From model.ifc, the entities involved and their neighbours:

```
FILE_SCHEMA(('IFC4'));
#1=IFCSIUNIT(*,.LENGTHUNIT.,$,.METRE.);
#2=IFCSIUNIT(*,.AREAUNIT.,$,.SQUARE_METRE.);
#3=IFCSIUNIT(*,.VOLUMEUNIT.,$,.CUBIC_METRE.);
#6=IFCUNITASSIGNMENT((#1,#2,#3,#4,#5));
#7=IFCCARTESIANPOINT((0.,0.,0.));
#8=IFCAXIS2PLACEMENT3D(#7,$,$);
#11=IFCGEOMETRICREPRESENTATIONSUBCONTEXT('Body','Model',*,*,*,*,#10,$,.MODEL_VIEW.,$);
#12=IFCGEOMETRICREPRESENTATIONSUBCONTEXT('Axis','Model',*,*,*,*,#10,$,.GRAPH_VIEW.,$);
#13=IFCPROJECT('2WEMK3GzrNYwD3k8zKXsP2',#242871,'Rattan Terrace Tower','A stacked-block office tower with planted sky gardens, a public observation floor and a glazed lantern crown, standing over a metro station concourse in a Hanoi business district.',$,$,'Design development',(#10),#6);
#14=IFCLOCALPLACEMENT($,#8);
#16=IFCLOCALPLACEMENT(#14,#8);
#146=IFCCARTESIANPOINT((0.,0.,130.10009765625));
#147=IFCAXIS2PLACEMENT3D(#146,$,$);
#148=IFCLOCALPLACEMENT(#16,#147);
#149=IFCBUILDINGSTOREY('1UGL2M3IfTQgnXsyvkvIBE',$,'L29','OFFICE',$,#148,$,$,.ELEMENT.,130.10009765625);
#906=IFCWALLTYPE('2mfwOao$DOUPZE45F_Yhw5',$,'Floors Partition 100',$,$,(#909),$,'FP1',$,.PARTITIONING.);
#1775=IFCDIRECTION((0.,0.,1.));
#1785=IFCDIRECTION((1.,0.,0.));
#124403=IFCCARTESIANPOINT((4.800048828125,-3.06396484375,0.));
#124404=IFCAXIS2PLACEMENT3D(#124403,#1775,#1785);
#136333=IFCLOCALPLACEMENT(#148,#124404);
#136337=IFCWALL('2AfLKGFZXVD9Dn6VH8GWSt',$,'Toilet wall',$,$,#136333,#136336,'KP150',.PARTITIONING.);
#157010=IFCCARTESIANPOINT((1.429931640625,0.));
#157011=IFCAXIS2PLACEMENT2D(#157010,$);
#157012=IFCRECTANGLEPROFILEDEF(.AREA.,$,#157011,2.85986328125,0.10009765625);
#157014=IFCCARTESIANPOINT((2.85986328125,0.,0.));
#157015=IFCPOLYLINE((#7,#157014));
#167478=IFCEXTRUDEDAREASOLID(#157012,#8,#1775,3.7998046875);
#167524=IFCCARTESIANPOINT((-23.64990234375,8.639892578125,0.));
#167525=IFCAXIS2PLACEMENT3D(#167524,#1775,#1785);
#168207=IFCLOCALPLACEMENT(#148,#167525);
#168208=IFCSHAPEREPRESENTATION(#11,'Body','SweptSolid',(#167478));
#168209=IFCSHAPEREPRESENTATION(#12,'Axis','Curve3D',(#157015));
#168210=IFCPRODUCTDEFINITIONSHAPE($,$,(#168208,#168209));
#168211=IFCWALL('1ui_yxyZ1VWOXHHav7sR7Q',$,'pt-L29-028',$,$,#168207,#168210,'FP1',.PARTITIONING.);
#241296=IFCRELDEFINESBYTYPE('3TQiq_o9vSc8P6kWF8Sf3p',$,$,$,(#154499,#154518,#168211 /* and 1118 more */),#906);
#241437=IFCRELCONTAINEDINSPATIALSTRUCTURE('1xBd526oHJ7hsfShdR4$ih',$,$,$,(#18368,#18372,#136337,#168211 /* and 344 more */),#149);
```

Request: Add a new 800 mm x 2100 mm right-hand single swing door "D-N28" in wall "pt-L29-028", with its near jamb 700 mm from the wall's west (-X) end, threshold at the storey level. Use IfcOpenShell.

```python
import numpy as np
import ifcopenshell
import ifcopenshell.api.feature
import ifcopenshell.api.geometry
import ifcopenshell.api.root
import ifcopenshell.api.spatial
import ifcopenshell.geom
import ifcopenshell.util.element
import ifcopenshell.util.placement
import ifcopenshell.util.representation
import ifcopenshell.util.shape
import ifcopenshell.util.unit

model = ifcopenshell.open("model.ifc")
unit_scale = ifcopenshell.util.unit.calculate_unit_scale(model)
settings = ifcopenshell.geom.settings()


def volume(element):
    """Net volume in cubic metres, openings subtracted."""
    shape = ifcopenshell.geom.create_shape(settings, element)
    return ifcopenshell.util.shape.get_volume(shape.geometry)


wall = model.by_guid("1ui_yxyZ1VWOXHHav7sR7Q")
storey = ifcopenshell.util.element.get_container(wall, ifc_class="IfcBuildingStorey")
context = ifcopenshell.util.representation.get_context(model, "Model", "Body", "MODEL_VIEW")
before = volume(wall)

width, height, from_end, sill = 0.8, 2.1, 0.7, 0.0  # metres

# The wall runs along its own X axis, and the end named is its -X end.
wall_shape = ifcopenshell.geom.create_shape(settings, wall)
x, y, z = ifcopenshell.util.shape.get_vertices(wall_shape.geometry).T
start = x.min() + from_end
face, thickness = float(y.min()), float(y.max() - y.min())
wall_matrix = ifcopenshell.util.placement.get_local_placement(wall.ObjectPlacement)
level = ifcopenshell.util.placement.get_local_placement(storey.ObjectPlacement)[2, 3]


def in_wall(x, y):
    """Placement at x, y metres in the wall's axes, at sill height."""
    matrix = wall_matrix.copy()
    matrix[:, 3] = wall_matrix @ np.array([x / unit_scale, y / unit_scale, 0.0, 1.0])
    matrix[2, 3] = level + sill / unit_scale
    return matrix


# Opening: a box that overshoots both wall faces by 50 mm.
opening = ifcopenshell.api.root.create_entity(model, ifc_class="IfcOpeningElement", predefined_type="OPENING")
box = ifcopenshell.api.geometry.add_wall_representation(
    model, context=context, length=width, height=height, thickness=thickness + 0.1
)
ifcopenshell.api.geometry.assign_representation(model, product=opening, representation=box)
ifcopenshell.api.geometry.edit_object_placement(model, product=opening, matrix=in_wall(start, face - 0.05), is_si=False)
ifcopenshell.api.feature.add_feature(model, feature=opening, element=wall)

door = ifcopenshell.api.root.create_entity(model, ifc_class="IfcDoor", name="D-N28", predefined_type="DOOR")
door.OverallWidth, door.OverallHeight = width / unit_scale, height / unit_scale
door.OperationType = "SINGLE_SWING_RIGHT"
body = ifcopenshell.api.geometry.add_door_representation(
    model,
    context=context,
    overall_width=door.OverallWidth,
    overall_height=door.OverallHeight,
    operation_type="SINGLE_SWING_RIGHT",
    lining_properties={"LiningDepth": thickness / unit_scale, "ThresholdDepth": thickness / unit_scale},
)
ifcopenshell.api.geometry.assign_representation(model, product=door, representation=body)
ifcopenshell.api.spatial.assign_container(model, products=[door], relating_structure=storey)
ifcopenshell.api.feature.add_filling(model, opening=opening, element=door)

# The lining spans the wall, so the door starts at the wall face.
ifcopenshell.api.geometry.edit_object_placement(model, product=door, matrix=in_wall(start, face), is_si=False)

after = volume(wall)

print(f"wall volume {before:.3f} -> {after:.3f} m3")

model.write("model_rev.ifc")
```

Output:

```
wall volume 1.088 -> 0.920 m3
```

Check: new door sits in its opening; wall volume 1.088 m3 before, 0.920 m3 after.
